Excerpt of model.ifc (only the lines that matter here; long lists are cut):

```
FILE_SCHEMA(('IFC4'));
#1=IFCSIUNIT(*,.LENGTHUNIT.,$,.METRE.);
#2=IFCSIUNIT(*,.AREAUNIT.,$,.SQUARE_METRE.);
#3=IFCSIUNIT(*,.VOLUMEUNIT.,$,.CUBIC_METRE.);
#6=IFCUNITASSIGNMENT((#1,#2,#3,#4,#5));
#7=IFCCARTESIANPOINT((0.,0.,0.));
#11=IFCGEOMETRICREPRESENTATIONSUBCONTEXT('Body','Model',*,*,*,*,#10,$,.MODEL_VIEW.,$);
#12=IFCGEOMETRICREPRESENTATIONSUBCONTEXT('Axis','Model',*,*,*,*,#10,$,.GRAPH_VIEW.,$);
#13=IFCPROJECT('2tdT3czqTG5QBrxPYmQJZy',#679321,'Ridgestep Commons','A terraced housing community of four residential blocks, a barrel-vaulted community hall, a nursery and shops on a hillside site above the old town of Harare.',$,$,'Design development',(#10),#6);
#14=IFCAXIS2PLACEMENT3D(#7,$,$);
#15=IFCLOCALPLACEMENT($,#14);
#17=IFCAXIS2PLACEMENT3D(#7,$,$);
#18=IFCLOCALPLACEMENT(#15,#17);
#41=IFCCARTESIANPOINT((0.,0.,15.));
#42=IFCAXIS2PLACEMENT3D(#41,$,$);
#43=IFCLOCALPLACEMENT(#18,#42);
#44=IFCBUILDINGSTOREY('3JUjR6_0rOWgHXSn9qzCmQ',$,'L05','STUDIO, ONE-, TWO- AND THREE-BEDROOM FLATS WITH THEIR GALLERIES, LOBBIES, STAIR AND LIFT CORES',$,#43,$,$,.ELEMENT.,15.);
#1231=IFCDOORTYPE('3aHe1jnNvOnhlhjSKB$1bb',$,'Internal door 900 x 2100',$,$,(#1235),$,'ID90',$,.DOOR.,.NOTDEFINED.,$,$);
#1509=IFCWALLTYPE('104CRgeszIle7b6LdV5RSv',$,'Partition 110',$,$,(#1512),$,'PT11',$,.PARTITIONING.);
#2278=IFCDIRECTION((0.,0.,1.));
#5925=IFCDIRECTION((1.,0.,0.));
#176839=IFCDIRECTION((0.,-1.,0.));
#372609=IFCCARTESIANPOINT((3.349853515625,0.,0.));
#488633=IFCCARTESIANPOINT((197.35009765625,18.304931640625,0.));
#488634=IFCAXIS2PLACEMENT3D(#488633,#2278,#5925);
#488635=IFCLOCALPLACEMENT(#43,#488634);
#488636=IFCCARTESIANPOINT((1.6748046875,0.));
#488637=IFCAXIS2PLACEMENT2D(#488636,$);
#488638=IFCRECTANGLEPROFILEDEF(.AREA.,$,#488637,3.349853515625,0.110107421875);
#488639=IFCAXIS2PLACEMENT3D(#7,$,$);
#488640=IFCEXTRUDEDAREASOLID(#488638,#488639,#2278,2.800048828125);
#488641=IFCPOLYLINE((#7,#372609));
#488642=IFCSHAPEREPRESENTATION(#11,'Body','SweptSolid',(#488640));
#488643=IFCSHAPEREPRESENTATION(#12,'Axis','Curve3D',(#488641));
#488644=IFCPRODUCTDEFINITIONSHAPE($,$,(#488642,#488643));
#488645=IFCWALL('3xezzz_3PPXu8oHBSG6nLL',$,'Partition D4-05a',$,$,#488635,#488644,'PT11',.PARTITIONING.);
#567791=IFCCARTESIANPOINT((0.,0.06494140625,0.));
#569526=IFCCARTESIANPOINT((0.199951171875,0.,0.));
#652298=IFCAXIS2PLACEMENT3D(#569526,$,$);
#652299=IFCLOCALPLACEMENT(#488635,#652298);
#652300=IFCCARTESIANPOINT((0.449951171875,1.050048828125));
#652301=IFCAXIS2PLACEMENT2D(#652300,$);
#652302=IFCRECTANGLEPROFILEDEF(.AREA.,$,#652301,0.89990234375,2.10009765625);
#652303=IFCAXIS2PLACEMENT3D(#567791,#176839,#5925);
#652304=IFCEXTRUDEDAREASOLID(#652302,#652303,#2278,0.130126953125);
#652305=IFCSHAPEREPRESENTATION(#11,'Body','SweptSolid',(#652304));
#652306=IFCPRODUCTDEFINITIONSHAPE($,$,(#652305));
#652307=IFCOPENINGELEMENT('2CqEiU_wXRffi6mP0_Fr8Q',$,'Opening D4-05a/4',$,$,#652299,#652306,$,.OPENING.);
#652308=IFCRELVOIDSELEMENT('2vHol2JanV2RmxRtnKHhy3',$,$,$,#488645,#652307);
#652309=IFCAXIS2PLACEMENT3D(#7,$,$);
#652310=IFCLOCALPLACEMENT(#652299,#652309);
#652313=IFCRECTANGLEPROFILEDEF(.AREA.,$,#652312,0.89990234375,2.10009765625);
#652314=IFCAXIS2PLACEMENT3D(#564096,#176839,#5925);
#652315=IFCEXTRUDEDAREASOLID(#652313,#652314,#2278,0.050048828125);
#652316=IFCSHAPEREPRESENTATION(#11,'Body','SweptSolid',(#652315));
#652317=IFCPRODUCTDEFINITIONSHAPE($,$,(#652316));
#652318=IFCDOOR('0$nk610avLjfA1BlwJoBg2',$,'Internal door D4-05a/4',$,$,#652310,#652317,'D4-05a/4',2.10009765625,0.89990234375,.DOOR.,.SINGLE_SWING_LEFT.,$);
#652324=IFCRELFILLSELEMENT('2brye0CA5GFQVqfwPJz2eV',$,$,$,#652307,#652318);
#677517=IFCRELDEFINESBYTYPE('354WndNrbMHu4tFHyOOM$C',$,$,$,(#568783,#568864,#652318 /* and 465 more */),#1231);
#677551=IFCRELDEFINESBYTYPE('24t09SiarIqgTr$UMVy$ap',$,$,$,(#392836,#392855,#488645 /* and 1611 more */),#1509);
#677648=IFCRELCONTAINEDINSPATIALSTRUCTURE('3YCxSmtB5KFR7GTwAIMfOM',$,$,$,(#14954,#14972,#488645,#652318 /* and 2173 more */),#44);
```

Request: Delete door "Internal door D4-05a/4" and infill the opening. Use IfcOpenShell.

```python
import ifcopenshell
import ifcopenshell.api.feature
import ifcopenshell.api.root
import ifcopenshell.geom
import ifcopenshell.util.shape

model = ifcopenshell.open("model.ifc")
settings = ifcopenshell.geom.settings()


def volume(element):
    """Net volume in cubic metres, openings subtracted."""
    shape = ifcopenshell.geom.create_shape(settings, element)
    return ifcopenshell.util.shape.get_volume(shape.geometry)


door = model.by_id(652318)
opening = door.FillsVoids[0].RelatingOpeningElement
wall = opening.VoidsElements[0].RelatingBuildingElement
before = volume(wall)

ifcopenshell.api.root.remove_product(model, product=door)
ifcopenshell.api.feature.remove_feature(model, feature=opening)

after = volume(wall)

print(f"wall volume {before:.3f} -> {after:.3f} m3")

model.write("model_v2.ifc")
```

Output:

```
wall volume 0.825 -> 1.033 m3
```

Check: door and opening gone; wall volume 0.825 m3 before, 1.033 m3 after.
